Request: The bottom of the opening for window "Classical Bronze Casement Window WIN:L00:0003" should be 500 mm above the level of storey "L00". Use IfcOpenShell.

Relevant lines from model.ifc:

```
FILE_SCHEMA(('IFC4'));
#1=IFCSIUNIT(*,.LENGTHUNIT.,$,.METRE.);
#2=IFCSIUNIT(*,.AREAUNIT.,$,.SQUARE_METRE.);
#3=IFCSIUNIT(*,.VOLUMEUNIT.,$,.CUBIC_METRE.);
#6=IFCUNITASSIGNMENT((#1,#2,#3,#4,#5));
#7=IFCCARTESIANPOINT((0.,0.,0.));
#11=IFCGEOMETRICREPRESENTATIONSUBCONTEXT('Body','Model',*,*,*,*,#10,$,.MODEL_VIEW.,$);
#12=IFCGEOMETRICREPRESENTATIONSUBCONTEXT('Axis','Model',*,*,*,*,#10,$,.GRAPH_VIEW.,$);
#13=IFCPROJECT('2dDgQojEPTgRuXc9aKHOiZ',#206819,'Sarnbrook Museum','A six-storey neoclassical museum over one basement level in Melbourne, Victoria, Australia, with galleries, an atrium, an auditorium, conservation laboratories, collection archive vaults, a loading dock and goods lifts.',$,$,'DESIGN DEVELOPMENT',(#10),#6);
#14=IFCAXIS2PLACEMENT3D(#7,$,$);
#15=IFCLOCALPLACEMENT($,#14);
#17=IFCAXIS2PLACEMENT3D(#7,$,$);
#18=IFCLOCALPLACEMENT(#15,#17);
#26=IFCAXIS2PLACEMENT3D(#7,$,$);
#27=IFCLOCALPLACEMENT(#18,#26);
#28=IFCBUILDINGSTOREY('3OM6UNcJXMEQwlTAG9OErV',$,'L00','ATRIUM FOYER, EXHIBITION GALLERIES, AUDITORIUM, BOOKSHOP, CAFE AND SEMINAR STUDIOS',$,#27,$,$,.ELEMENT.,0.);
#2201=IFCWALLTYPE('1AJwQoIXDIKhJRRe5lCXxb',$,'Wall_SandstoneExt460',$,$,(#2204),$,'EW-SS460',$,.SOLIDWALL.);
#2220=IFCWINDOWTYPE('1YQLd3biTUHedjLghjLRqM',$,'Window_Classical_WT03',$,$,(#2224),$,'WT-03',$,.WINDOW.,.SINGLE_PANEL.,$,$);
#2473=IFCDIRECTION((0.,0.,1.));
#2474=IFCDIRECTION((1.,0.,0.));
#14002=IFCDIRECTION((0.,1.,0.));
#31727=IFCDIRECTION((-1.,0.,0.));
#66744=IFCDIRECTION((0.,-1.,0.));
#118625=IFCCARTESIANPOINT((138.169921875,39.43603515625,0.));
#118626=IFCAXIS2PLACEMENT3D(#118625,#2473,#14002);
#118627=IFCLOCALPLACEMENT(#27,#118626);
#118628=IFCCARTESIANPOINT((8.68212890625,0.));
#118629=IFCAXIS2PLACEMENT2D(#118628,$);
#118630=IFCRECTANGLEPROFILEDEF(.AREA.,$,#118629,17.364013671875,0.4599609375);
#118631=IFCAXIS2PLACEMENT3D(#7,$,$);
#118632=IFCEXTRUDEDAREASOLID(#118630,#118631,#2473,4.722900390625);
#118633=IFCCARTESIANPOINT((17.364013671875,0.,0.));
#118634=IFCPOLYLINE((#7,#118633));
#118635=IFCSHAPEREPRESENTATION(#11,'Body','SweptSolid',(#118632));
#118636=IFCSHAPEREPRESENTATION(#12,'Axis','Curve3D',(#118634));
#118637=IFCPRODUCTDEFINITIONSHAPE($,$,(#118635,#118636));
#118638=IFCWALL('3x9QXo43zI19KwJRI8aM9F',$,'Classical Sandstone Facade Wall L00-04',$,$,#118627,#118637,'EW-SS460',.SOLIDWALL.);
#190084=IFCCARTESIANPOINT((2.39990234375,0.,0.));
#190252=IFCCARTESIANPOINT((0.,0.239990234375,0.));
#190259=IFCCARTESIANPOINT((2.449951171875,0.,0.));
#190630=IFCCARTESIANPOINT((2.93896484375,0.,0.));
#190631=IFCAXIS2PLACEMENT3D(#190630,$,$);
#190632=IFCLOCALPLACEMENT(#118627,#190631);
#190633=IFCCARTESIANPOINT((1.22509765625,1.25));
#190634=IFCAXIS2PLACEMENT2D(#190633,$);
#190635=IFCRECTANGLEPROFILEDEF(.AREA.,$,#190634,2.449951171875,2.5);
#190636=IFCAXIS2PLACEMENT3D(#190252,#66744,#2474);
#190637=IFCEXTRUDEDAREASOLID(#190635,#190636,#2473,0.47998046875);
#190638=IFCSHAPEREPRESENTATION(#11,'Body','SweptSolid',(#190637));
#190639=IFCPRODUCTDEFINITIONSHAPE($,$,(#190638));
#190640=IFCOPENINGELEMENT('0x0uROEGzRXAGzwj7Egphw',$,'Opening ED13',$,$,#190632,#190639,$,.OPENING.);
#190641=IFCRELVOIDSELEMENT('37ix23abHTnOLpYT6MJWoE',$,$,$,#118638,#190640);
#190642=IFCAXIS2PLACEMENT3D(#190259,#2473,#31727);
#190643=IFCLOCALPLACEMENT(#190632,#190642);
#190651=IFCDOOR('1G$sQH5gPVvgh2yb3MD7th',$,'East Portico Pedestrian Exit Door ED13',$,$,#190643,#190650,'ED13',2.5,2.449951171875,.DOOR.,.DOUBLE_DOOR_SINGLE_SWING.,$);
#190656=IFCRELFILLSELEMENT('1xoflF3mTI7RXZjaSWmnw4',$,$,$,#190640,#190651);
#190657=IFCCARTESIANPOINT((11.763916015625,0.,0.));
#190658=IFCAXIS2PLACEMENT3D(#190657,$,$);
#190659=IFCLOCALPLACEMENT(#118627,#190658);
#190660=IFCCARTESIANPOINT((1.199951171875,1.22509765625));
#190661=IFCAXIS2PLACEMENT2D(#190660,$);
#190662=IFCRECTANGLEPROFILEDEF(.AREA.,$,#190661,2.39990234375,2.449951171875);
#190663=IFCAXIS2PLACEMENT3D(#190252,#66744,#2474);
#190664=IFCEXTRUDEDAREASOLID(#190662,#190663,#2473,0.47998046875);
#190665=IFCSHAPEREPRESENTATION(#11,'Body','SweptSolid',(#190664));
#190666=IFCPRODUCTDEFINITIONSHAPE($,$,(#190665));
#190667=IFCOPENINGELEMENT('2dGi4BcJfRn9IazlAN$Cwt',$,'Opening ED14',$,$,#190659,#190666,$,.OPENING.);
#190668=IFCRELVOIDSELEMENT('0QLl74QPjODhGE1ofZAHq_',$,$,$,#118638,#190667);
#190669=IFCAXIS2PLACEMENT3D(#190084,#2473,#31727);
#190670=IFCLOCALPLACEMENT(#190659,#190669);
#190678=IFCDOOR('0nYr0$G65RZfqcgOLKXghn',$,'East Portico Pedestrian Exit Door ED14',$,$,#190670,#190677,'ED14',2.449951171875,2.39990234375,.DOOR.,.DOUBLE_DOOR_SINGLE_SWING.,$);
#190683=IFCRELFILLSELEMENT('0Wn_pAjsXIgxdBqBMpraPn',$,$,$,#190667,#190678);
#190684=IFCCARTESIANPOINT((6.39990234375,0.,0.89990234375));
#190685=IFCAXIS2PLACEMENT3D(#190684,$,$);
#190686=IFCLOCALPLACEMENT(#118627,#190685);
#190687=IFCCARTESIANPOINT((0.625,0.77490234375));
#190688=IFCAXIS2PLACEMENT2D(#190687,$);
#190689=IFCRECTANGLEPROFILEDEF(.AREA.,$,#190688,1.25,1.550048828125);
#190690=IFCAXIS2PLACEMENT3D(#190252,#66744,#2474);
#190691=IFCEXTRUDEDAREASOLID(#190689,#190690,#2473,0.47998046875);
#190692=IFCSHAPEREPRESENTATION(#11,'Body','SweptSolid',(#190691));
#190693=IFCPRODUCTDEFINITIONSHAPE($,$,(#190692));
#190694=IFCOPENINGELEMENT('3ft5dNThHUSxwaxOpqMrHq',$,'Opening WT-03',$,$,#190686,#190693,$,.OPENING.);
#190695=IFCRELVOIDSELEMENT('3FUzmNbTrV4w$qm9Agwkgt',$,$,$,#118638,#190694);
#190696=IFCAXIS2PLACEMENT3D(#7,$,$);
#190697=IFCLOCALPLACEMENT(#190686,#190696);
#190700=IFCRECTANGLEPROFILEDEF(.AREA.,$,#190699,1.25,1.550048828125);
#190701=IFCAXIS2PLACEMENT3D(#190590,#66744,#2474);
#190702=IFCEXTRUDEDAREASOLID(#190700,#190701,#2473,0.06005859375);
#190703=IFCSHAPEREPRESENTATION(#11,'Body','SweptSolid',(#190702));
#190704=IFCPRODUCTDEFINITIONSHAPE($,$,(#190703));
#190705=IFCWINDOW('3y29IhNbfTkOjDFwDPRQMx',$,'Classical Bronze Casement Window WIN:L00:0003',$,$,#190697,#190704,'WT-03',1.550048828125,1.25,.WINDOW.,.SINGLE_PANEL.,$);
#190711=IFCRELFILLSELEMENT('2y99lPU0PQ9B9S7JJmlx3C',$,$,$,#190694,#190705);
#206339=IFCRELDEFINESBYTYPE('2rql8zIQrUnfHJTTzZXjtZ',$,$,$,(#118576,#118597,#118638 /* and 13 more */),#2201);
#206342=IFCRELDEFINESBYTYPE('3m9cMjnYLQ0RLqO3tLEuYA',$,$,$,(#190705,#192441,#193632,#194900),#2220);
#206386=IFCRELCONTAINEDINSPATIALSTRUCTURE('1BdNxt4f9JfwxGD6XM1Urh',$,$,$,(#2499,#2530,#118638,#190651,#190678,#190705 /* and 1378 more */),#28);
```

```python
import numpy as np
import ifcopenshell
import ifcopenshell.api.geometry
import ifcopenshell.geom
import ifcopenshell.util.element
import ifcopenshell.util.placement
import ifcopenshell.util.shape
import ifcopenshell.util.unit

model = ifcopenshell.open("model.ifc")
unit_scale = ifcopenshell.util.unit.calculate_unit_scale(model)

window = model.by_id(190705)
opening = window.FillsVoids[0].RelatingOpeningElement
storey = ifcopenshell.util.element.get_container(window, ifc_class="IfcBuildingStorey")
level = ifcopenshell.util.placement.get_local_placement(storey.ObjectPlacement)[2, 3]

# The opening's origin need not be at the sill, so measure its lowest point.
shape = ifcopenshell.geom.create_shape(ifcopenshell.geom.settings(), opening)
bottom = ifcopenshell.util.shape.get_shape_bottom_elevation(shape, shape.geometry) / unit_scale
dz = level + 0.5 / unit_scale - bottom

shift = np.array([0.0, 0.0, dz])
# The window is placed relative to its opening, so it follows when the opening moves.
matrix = ifcopenshell.util.placement.get_local_placement(opening.ObjectPlacement)
matrix[:3, 3] += shift
ifcopenshell.api.geometry.edit_object_placement(
    model, product=opening, matrix=matrix, is_si=False, should_transform_children=True
)

print(f"moved by {dz * unit_scale:+.3f} m")

model.write("model_v2.ifc")
```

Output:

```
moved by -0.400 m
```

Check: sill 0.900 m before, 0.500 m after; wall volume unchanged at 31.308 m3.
